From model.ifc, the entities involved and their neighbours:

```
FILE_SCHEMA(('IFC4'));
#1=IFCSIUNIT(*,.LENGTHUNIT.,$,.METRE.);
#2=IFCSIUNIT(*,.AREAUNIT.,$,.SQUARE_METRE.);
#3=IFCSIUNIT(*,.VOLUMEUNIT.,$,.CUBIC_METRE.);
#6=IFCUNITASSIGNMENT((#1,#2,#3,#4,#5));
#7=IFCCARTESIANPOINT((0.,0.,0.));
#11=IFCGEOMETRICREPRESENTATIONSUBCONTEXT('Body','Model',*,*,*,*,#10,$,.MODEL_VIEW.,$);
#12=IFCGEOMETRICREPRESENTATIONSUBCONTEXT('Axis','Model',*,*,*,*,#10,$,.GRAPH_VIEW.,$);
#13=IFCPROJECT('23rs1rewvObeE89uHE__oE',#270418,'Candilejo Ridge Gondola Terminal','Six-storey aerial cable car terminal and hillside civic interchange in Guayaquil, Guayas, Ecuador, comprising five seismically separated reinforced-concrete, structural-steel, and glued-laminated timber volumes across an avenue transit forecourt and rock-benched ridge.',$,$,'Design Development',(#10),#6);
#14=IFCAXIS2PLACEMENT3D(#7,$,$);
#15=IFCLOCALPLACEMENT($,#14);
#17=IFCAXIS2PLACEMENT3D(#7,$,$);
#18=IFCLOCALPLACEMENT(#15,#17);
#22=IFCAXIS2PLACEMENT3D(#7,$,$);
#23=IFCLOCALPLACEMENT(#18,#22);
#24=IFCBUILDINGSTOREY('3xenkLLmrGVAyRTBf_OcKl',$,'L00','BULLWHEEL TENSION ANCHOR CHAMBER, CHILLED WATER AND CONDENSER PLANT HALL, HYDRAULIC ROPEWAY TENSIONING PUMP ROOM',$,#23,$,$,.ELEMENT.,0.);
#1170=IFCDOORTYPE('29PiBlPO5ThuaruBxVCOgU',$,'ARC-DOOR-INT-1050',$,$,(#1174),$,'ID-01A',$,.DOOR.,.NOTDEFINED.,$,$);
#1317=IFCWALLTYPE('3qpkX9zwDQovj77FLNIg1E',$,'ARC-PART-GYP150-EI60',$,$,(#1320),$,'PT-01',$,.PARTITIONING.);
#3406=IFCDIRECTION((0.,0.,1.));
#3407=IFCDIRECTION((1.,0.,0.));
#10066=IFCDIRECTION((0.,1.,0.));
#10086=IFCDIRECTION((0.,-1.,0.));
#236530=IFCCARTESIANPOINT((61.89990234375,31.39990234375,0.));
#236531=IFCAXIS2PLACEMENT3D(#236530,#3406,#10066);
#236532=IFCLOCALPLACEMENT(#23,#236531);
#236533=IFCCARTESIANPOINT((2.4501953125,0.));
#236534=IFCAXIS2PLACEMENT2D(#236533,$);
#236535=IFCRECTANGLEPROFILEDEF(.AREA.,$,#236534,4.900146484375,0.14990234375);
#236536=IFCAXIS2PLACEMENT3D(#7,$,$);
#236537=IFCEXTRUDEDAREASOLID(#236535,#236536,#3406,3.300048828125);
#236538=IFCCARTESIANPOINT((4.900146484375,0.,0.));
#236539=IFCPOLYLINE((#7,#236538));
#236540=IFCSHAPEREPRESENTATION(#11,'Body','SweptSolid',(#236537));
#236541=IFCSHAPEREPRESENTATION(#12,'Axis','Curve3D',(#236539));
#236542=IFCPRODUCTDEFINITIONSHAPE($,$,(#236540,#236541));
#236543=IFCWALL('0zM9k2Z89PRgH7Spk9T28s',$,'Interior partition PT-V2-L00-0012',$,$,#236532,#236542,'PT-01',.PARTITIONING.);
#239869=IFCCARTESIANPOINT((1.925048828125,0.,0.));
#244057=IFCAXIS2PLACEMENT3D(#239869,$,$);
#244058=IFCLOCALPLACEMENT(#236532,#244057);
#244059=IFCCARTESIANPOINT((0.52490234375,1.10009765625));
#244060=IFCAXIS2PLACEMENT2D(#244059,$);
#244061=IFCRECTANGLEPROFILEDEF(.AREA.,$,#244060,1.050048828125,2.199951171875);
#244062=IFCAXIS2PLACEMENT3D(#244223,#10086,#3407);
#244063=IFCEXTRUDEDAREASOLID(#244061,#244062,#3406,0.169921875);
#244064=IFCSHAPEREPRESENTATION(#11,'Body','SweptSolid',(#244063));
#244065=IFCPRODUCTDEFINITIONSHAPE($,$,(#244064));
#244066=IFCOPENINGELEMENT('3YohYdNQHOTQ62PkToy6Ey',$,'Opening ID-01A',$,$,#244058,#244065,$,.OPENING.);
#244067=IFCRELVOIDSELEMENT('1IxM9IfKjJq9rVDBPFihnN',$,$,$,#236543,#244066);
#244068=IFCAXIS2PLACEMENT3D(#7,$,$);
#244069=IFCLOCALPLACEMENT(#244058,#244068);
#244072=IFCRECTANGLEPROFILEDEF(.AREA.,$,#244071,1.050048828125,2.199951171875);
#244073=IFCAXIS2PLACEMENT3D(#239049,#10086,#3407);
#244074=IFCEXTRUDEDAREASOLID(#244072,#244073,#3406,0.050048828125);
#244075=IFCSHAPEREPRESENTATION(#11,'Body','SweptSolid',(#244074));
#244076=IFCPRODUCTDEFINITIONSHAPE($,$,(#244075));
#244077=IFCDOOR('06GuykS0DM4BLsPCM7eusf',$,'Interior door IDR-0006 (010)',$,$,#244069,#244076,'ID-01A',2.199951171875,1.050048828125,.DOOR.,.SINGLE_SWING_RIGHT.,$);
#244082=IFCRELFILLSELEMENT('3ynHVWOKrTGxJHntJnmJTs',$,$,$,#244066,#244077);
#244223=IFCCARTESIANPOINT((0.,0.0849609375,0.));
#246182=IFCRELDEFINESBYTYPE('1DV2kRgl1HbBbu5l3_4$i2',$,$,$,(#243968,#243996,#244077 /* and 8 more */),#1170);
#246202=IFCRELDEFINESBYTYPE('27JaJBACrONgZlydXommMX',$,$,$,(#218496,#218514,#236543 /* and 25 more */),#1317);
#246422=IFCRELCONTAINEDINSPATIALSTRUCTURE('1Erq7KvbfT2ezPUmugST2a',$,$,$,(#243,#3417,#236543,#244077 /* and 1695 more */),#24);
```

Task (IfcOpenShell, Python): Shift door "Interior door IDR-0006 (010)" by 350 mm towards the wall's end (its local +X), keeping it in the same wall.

```python
import ifcopenshell
import ifcopenshell.api.geometry
import ifcopenshell.util.placement
import ifcopenshell.util.unit

model = ifcopenshell.open("model.ifc")
unit_scale = ifcopenshell.util.unit.calculate_unit_scale(model)

door = model.by_guid("06GuykS0DM4BLsPCM7eusf")
opening = door.FillsVoids[0].RelatingOpeningElement
wall = opening.VoidsElements[0].RelatingBuildingElement

wall_matrix = ifcopenshell.util.placement.get_local_placement(wall.ObjectPlacement)
shift = wall_matrix[:3, 0] * 0.35 / unit_scale
before = ifcopenshell.util.placement.get_local_placement(door.ObjectPlacement)[:3, 3].copy()

# The door is placed relative to its opening, so it follows when the opening moves.
matrix = ifcopenshell.util.placement.get_local_placement(opening.ObjectPlacement)
matrix[:3, 3] += shift
ifcopenshell.api.geometry.edit_object_placement(
    model, product=opening, matrix=matrix, is_si=False, should_transform_children=True
)

after = ifcopenshell.util.placement.get_local_placement(door.ObjectPlacement)[:3, 3]
print("door moved by", (after - before).round(3) + 0.0)

model.write("model_v2.ifc")
```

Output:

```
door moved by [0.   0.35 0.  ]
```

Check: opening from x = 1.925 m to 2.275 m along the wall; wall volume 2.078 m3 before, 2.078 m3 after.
